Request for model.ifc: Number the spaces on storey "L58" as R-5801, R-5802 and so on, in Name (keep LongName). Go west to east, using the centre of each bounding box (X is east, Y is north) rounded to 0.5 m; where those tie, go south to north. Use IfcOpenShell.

First a look at what the model holds.

```python
import ifcopenshell
import ifcopenshell.util.element
import ifcopenshell.util.placement

model = ifcopenshell.open("model.ifc")
print(model.schema)
storey = next(s for s in model.by_type("IfcBuildingStorey") if s.Name == "L58")
spaces = [e for e in ifcopenshell.util.element.get_decomposition(storey) if e.is_a("IfcSpace")]
for e in sorted(spaces, key=lambda e: e.id()):
    origin = ifcopenshell.util.placement.get_local_placement(e.ObjectPlacement)[:3, 3]
    print(e.id(), e.Name, e.LongName, origin.round(2) + 0.0, sep=" | ")
```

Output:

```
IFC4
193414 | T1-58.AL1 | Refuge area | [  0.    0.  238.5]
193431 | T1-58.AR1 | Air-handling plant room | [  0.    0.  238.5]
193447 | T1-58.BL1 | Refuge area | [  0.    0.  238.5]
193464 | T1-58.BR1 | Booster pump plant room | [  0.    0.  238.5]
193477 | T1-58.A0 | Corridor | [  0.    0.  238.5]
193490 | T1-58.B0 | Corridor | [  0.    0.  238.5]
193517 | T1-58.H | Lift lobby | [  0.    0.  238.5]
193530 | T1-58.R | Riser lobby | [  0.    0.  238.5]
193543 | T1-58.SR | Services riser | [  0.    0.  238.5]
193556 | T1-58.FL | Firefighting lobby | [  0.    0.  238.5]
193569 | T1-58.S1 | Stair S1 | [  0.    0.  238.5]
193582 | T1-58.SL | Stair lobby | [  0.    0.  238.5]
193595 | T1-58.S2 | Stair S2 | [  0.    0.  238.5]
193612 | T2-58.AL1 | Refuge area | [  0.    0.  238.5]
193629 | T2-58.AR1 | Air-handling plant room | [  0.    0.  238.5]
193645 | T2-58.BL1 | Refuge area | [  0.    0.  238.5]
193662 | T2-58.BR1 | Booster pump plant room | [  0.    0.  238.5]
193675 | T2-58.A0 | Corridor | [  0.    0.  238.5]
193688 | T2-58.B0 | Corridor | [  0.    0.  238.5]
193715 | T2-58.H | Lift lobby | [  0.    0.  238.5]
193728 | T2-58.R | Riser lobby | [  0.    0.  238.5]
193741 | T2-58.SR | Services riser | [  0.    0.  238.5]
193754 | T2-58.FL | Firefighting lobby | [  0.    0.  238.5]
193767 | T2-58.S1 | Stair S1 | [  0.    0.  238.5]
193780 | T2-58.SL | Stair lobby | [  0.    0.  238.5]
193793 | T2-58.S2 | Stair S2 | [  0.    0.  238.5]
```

```python
import ifcopenshell
import ifcopenshell.geom
import ifcopenshell.util.element
import ifcopenshell.util.shape

model = ifcopenshell.open("model.ifc")
settings = ifcopenshell.geom.settings()
settings.set("use-world-coords", True)


def centre(element):
    shape = ifcopenshell.geom.create_shape(settings, element)
    return ifcopenshell.util.shape.get_bbox_centroid(shape.geometry)


storey = next(s for s in model.by_type("IfcBuildingStorey") if s.Name == "L58")
spaces = [e for e in ifcopenshell.util.element.get_decomposition(storey) if e.is_a("IfcSpace")]

# Insertion points can sit at a corner or the storey origin, so sort by the geometry (in metres).
centres = {e: centre(e) for e in spaces}
spaces.sort(key=lambda e: (round(centres[e][0] / 0.5), centres[e][1]))

for i, e in enumerate(spaces, start=1):
    number = f"R-58{i:02d}"
    e.Name = number
    print(e.id(), number)

model.write("model_edited.ifc")
```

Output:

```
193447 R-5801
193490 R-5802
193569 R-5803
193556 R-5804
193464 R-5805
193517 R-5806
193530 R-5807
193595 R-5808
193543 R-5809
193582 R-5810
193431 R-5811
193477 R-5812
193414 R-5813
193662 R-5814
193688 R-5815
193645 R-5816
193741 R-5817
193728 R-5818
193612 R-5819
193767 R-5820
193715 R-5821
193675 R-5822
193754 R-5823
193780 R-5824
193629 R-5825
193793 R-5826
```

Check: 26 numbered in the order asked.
